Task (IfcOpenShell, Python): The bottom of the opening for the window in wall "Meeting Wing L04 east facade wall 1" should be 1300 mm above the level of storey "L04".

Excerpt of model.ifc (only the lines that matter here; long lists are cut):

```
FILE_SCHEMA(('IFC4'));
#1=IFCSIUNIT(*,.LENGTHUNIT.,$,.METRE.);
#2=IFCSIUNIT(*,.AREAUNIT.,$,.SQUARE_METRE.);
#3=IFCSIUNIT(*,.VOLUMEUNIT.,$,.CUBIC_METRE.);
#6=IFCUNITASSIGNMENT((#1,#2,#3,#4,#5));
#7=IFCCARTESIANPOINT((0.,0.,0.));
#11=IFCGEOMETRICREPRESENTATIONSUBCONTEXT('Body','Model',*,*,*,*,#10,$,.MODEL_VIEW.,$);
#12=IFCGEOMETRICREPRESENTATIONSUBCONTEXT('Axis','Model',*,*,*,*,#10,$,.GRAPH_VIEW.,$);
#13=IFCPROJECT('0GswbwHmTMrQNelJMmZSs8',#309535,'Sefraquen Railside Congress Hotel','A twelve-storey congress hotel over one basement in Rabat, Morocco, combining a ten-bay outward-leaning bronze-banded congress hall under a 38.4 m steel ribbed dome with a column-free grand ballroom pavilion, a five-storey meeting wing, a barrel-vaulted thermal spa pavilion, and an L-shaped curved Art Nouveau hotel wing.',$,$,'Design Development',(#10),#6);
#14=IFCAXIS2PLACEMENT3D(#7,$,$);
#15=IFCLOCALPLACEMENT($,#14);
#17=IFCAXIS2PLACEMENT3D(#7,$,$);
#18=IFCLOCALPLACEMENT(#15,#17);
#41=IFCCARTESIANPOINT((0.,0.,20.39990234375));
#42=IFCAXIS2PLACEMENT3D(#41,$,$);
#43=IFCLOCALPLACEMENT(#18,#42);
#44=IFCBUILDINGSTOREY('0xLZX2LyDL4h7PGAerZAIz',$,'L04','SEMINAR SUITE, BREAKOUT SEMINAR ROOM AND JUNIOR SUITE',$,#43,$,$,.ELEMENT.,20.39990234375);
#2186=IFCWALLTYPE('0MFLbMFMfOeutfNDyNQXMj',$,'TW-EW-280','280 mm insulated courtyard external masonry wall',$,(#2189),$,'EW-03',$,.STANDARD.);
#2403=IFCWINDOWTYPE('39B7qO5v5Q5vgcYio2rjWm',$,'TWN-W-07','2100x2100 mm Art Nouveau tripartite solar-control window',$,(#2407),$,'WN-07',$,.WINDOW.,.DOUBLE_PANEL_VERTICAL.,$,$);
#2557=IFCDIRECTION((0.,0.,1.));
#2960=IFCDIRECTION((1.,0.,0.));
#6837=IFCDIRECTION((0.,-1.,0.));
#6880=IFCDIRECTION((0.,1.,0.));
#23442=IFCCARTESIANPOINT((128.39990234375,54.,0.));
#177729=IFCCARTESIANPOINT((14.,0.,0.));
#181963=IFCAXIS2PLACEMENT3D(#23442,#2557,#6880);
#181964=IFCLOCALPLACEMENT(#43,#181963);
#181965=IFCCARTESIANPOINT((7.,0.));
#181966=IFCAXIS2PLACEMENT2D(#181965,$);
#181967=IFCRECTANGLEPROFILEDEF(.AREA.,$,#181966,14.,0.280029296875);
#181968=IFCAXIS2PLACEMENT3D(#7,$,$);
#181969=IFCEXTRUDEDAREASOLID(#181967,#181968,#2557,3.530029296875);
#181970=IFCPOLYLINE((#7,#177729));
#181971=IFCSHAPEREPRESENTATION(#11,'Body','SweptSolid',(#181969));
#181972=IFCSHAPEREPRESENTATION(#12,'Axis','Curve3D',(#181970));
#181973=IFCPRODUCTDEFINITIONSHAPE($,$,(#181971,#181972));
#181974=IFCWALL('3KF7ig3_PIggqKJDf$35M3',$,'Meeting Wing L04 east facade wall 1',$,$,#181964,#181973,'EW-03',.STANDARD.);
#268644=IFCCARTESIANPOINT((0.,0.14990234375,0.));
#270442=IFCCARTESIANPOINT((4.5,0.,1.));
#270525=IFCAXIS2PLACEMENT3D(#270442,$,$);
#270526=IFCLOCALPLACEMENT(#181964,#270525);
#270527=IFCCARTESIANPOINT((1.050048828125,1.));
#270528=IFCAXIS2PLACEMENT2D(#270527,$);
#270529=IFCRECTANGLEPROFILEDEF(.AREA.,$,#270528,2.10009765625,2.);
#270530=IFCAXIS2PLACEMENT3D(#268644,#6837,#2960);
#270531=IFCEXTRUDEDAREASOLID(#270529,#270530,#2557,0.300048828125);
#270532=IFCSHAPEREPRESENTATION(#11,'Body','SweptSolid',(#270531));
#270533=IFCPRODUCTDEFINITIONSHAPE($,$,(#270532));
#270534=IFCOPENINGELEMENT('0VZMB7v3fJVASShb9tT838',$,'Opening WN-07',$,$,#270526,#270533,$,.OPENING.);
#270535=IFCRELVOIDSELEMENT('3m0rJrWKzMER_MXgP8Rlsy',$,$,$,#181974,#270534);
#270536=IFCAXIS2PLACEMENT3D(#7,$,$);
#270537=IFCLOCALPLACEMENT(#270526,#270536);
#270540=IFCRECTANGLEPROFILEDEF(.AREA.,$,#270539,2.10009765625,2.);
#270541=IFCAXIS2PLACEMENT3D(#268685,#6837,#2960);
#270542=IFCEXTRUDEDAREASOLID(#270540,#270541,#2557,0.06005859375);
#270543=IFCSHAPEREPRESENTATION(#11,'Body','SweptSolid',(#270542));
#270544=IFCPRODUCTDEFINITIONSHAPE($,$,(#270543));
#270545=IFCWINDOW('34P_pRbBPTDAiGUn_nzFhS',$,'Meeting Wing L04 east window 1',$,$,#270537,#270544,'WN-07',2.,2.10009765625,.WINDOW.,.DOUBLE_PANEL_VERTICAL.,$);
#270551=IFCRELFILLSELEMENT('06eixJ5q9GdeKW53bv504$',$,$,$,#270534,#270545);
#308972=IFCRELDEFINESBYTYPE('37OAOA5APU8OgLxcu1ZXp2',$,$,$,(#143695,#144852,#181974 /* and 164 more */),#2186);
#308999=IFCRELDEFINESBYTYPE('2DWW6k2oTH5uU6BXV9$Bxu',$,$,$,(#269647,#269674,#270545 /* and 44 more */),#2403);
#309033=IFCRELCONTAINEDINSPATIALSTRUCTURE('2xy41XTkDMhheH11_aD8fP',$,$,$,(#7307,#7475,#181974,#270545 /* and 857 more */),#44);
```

```python
import numpy as np
import ifcopenshell
import ifcopenshell.api.geometry
import ifcopenshell.geom
import ifcopenshell.util.element
import ifcopenshell.util.placement
import ifcopenshell.util.shape
import ifcopenshell.util.unit

model = ifcopenshell.open("model.ifc")
unit_scale = ifcopenshell.util.unit.calculate_unit_scale(model)

window = model.by_guid("34P_pRbBPTDAiGUn_nzFhS")
opening = window.FillsVoids[0].RelatingOpeningElement
storey = ifcopenshell.util.element.get_container(window, ifc_class="IfcBuildingStorey")
level = ifcopenshell.util.placement.get_local_placement(storey.ObjectPlacement)[2, 3]

# The opening's origin need not be at the sill, so measure its lowest point.
shape = ifcopenshell.geom.create_shape(ifcopenshell.geom.settings(), opening)
bottom = ifcopenshell.util.shape.get_shape_bottom_elevation(shape, shape.geometry) / unit_scale
dz = level + 1.3 / unit_scale - bottom

shift = np.array([0.0, 0.0, dz])
# The window is placed relative to its opening, so it follows when the opening moves.
matrix = ifcopenshell.util.placement.get_local_placement(opening.ObjectPlacement)
matrix[:3, 3] += shift
ifcopenshell.api.geometry.edit_object_placement(
    model, product=opening, matrix=matrix, is_si=False, should_transform_children=True
)

print(f"moved by {dz * unit_scale:+.3f} m")

model.write("model_updated.ifc")
```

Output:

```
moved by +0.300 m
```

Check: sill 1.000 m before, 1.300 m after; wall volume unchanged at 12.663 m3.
